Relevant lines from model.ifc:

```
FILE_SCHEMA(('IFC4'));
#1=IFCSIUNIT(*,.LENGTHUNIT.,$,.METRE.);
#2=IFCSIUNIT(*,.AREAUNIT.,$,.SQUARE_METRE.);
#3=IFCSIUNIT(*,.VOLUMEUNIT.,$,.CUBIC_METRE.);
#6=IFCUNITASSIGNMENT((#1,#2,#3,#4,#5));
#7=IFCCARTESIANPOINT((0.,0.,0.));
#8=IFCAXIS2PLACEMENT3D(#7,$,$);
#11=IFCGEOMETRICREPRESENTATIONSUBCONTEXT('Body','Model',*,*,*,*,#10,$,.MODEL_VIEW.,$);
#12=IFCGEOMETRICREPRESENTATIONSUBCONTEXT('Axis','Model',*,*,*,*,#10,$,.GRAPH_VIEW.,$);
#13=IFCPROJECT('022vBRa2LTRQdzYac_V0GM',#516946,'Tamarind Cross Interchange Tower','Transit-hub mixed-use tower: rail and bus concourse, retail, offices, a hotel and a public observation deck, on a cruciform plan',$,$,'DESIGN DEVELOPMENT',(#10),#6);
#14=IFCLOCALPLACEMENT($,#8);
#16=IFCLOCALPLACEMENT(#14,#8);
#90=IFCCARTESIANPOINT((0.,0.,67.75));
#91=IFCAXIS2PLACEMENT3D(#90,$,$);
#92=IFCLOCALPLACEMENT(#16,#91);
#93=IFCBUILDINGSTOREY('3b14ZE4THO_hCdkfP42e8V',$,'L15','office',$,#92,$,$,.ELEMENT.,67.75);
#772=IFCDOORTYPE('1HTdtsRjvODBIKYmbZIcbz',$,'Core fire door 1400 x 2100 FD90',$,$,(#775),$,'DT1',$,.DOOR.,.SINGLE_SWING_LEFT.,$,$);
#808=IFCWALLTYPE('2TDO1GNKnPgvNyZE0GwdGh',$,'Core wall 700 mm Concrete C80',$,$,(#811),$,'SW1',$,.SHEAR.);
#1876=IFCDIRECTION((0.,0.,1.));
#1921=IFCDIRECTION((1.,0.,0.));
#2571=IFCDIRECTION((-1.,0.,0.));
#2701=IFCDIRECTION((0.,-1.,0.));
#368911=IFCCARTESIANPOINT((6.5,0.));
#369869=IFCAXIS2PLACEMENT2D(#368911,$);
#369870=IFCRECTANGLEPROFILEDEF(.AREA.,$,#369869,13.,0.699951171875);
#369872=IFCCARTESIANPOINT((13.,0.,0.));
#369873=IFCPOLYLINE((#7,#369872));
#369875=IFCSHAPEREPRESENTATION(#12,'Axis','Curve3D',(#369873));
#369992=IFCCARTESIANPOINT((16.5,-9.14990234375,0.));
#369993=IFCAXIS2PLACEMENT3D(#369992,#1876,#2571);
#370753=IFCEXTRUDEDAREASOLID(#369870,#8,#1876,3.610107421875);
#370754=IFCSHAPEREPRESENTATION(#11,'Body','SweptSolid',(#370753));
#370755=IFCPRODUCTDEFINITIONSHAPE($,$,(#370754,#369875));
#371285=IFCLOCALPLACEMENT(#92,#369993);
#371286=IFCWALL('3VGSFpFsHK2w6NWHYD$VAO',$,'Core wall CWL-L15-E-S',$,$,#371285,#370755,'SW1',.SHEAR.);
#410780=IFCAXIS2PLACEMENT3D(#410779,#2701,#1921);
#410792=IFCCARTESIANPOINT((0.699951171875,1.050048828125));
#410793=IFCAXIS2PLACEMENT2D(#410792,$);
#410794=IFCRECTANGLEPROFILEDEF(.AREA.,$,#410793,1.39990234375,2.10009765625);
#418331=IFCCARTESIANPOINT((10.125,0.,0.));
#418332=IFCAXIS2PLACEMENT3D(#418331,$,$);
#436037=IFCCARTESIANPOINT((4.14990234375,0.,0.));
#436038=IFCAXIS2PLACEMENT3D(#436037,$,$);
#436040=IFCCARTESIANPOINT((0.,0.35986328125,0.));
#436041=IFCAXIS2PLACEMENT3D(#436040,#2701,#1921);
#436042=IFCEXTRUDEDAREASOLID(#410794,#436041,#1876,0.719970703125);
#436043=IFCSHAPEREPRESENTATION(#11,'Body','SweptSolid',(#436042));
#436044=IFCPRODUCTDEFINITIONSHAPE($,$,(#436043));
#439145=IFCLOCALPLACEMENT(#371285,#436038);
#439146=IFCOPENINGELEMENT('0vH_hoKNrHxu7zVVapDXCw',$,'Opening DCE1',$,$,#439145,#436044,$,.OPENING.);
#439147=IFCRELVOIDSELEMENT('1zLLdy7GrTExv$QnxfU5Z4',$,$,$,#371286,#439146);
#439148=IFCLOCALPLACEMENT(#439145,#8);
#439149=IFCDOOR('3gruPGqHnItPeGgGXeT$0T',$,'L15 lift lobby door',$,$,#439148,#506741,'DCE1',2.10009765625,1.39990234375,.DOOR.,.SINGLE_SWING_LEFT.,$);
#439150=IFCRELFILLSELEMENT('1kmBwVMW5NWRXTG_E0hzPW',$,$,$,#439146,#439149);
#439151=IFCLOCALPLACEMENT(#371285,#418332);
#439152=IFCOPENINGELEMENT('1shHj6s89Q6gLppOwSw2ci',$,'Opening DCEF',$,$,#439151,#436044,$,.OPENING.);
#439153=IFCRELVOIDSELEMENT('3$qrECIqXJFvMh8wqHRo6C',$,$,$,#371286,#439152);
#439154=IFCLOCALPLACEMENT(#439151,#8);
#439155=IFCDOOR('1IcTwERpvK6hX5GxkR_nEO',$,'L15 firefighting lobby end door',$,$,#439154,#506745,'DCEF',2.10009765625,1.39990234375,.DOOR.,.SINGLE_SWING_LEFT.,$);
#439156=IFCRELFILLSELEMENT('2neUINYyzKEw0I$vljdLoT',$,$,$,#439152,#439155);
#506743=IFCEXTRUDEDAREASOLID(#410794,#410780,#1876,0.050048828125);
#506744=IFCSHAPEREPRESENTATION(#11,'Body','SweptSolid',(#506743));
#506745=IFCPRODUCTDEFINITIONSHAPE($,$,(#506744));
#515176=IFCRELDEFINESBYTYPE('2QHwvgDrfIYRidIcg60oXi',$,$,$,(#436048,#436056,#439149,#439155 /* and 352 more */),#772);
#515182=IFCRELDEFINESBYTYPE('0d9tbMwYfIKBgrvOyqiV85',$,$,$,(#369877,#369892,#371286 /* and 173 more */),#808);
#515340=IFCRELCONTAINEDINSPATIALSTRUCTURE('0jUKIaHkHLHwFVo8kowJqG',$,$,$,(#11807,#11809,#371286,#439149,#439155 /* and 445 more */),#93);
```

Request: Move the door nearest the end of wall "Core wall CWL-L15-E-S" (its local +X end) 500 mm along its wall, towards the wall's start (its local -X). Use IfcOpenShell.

```python
import ifcopenshell
import ifcopenshell.api.geometry
import ifcopenshell.util.placement
import ifcopenshell.util.unit

model = ifcopenshell.open("model.ifc")
unit_scale = ifcopenshell.util.unit.calculate_unit_scale(model)

door = model.by_guid("1IcTwERpvK6hX5GxkR_nEO")
opening = door.FillsVoids[0].RelatingOpeningElement
wall = opening.VoidsElements[0].RelatingBuildingElement

wall_matrix = ifcopenshell.util.placement.get_local_placement(wall.ObjectPlacement)
shift = wall_matrix[:3, 0] * -0.5 / unit_scale
before = ifcopenshell.util.placement.get_local_placement(door.ObjectPlacement)[:3, 3].copy()

# The door is placed relative to its opening, so it follows when the opening moves.
matrix = ifcopenshell.util.placement.get_local_placement(opening.ObjectPlacement)
matrix[:3, 3] += shift
ifcopenshell.api.geometry.edit_object_placement(
    model, product=opening, matrix=matrix, is_si=False, should_transform_children=True
)

after = ifcopenshell.util.placement.get_local_placement(door.ObjectPlacement)[:3, 3]
print("door moved by", (after - before).round(3) + 0.0)

model.write("model_rev.ifc")
```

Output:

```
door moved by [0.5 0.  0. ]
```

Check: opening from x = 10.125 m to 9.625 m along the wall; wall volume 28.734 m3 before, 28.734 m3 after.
